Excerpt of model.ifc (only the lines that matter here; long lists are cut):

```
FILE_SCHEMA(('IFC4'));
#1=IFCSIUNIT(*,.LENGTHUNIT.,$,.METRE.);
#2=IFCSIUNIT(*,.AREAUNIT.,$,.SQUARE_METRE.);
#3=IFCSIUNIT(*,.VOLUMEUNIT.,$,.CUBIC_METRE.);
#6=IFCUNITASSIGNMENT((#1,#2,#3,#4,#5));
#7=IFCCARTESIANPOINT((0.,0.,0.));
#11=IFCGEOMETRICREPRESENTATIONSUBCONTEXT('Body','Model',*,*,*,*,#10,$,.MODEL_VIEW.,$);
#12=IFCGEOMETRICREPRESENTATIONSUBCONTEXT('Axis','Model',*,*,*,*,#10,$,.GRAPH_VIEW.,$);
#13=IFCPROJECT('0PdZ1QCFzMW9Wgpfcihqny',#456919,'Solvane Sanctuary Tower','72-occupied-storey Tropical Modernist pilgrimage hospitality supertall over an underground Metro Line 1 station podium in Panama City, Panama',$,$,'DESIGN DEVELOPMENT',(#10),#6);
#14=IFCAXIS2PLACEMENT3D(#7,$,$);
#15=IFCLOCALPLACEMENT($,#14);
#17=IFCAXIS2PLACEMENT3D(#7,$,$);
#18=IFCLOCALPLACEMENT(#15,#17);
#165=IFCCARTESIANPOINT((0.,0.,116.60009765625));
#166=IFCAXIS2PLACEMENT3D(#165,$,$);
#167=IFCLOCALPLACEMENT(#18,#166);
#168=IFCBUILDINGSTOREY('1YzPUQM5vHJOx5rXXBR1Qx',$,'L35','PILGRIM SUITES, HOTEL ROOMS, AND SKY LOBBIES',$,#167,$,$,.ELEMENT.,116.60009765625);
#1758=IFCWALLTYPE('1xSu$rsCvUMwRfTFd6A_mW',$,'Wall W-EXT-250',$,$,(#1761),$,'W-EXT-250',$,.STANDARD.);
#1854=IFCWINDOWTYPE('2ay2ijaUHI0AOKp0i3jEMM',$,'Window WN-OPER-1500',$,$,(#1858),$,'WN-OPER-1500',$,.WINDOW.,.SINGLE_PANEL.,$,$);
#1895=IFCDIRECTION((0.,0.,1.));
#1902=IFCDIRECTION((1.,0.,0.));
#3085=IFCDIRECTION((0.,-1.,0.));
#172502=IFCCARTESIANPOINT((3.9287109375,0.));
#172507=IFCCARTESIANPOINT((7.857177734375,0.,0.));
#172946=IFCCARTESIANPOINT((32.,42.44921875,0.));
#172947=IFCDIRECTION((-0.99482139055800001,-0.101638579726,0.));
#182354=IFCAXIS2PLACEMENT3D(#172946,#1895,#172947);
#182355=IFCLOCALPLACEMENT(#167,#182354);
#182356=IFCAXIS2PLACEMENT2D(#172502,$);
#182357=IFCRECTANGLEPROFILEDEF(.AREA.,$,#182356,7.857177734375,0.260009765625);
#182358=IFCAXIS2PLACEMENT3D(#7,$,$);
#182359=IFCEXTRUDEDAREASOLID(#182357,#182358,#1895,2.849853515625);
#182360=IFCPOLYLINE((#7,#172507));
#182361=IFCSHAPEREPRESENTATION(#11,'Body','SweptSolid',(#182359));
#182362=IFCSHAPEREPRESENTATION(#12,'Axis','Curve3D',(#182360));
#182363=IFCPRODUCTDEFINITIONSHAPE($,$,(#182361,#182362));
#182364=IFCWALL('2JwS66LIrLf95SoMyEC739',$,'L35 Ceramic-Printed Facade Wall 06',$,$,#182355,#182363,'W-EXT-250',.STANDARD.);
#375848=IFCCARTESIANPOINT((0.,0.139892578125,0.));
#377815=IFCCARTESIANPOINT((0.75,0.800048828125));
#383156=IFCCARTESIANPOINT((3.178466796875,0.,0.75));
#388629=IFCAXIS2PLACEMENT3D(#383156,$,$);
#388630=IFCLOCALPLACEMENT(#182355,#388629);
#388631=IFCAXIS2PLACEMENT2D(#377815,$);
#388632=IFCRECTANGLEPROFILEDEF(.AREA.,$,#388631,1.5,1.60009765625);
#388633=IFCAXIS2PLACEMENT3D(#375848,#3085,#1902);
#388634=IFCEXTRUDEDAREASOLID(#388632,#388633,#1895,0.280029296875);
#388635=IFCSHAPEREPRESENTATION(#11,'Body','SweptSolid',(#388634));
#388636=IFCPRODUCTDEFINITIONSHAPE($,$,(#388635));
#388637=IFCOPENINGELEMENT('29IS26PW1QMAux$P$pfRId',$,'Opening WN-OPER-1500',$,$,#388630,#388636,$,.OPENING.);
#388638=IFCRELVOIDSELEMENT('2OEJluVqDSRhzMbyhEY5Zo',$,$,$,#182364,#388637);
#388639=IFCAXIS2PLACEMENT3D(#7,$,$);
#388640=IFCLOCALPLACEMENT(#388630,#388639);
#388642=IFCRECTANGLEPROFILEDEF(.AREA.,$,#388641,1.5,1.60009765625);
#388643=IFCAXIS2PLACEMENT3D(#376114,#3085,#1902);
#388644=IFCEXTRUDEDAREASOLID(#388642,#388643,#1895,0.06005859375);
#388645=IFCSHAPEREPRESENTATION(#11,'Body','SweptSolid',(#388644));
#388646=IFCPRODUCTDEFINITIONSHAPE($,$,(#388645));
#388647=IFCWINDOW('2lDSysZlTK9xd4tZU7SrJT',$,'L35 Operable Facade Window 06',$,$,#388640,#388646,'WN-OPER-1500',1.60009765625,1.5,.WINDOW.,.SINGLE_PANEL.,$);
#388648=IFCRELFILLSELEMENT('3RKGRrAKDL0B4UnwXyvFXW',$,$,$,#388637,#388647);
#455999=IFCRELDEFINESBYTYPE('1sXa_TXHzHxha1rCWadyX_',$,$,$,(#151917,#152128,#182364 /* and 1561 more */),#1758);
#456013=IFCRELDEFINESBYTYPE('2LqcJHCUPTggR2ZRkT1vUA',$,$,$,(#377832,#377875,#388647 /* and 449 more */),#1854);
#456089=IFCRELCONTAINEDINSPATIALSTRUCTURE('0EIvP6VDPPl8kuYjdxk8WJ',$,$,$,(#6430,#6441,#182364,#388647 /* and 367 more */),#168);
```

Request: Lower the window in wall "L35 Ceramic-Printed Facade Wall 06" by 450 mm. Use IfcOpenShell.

```python
import numpy as np
import ifcopenshell
import ifcopenshell.api.geometry
import ifcopenshell.util.placement
import ifcopenshell.util.unit

model = ifcopenshell.open("model.ifc")
unit_scale = ifcopenshell.util.unit.calculate_unit_scale(model)

window = model.by_guid("2lDSysZlTK9xd4tZU7SrJT")
opening = window.FillsVoids[0].RelatingOpeningElement
dz = -0.45 / unit_scale

shift = np.array([0.0, 0.0, dz])
# The window is placed relative to its opening, so it follows when the opening moves.
matrix = ifcopenshell.util.placement.get_local_placement(opening.ObjectPlacement)
matrix[:3, 3] += shift
ifcopenshell.api.geometry.edit_object_placement(
    model, product=opening, matrix=matrix, is_si=False, should_transform_children=True
)

print(f"moved by {dz * unit_scale:+.3f} m")

model.write("model_rev.ifc")
```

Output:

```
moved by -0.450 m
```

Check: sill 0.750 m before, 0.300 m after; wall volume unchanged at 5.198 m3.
